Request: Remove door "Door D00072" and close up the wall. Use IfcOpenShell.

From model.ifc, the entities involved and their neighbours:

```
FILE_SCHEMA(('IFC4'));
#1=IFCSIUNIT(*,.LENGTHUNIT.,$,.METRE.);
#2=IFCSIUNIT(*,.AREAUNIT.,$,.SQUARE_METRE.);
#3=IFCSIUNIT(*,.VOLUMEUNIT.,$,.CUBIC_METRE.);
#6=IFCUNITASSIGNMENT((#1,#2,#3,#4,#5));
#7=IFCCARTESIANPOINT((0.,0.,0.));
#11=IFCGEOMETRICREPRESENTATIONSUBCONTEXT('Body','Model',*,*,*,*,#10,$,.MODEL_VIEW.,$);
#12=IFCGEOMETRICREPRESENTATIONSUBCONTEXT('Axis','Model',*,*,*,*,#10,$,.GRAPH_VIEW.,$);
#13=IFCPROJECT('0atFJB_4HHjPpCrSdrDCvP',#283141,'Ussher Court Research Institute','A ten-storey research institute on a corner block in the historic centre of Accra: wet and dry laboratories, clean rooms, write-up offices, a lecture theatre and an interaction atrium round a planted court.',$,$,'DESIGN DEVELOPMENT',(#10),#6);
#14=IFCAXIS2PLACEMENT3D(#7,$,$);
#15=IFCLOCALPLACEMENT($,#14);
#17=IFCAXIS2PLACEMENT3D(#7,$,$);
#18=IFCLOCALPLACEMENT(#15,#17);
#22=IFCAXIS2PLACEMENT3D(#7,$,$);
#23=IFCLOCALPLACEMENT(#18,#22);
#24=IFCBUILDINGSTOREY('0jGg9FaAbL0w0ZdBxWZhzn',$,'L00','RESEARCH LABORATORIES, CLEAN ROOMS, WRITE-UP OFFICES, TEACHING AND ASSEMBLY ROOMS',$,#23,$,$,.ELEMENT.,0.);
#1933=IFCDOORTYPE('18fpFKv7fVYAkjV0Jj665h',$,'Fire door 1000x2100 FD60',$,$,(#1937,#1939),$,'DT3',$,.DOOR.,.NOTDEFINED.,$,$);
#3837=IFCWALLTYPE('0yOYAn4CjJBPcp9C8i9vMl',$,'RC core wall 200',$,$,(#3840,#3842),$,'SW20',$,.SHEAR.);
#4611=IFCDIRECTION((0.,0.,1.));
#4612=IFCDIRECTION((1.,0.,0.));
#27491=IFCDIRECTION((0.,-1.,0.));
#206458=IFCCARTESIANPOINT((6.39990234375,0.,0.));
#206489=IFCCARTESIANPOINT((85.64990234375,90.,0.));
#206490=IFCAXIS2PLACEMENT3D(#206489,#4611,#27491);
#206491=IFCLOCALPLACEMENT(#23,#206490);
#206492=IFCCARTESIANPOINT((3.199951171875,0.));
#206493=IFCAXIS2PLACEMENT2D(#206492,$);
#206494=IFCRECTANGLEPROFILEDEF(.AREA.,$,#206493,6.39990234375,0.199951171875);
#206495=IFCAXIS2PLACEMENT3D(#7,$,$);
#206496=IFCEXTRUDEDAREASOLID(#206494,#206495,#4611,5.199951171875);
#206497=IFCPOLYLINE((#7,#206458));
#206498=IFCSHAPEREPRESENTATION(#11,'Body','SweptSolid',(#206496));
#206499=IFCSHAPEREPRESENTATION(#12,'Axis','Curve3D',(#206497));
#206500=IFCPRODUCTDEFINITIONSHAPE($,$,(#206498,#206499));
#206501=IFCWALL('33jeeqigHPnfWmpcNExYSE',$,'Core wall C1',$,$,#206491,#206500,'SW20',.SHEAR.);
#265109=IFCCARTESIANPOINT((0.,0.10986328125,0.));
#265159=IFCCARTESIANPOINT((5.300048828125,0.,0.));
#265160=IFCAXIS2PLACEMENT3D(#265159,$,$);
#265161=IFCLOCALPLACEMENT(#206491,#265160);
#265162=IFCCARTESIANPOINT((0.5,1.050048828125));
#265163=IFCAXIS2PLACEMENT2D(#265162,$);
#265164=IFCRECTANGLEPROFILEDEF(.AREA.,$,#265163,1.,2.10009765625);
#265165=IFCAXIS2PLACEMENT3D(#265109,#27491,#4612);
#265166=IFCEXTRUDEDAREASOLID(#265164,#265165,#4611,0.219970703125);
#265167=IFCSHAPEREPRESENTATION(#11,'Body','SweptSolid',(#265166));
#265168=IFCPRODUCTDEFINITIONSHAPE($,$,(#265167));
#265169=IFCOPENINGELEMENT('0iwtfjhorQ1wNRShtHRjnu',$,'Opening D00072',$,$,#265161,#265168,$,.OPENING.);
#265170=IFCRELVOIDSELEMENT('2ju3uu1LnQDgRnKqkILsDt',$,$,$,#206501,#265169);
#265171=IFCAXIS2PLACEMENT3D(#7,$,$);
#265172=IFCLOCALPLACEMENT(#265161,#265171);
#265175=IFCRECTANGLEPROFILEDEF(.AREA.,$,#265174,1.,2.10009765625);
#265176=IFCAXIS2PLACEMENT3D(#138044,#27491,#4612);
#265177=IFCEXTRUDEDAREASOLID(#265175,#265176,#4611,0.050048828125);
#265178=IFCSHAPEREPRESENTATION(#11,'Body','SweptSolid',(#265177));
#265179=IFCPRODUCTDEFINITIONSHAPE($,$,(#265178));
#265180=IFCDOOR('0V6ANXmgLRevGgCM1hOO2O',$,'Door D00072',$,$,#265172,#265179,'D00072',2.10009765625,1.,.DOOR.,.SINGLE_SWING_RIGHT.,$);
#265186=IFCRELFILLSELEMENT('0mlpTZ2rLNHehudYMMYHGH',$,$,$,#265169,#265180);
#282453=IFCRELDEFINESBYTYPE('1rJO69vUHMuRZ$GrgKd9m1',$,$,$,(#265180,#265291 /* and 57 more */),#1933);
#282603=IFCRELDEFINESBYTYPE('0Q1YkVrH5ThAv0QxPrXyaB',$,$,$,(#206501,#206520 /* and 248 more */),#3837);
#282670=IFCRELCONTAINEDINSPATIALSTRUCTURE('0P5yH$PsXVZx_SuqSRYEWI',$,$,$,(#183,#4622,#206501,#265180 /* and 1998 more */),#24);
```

```python
import ifcopenshell
import ifcopenshell.api.feature
import ifcopenshell.api.root
import ifcopenshell.geom
import ifcopenshell.util.shape

model = ifcopenshell.open("model.ifc")
settings = ifcopenshell.geom.settings()


def volume(element):
    """Net volume in cubic metres, openings subtracted."""
    shape = ifcopenshell.geom.create_shape(settings, element)
    return ifcopenshell.util.shape.get_volume(shape.geometry)


door = model.by_guid("0V6ANXmgLRevGgCM1hOO2O")
opening = door.FillsVoids[0].RelatingOpeningElement
wall = opening.VoidsElements[0].RelatingBuildingElement
before = volume(wall)

ifcopenshell.api.root.remove_product(model, product=door)
ifcopenshell.api.feature.remove_feature(model, feature=opening)

after = volume(wall)

print(f"wall volume {before:.3f} -> {after:.3f} m3")

model.write("model-out.ifc")
```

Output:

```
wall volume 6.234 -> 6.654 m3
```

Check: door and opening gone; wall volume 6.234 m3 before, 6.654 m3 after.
